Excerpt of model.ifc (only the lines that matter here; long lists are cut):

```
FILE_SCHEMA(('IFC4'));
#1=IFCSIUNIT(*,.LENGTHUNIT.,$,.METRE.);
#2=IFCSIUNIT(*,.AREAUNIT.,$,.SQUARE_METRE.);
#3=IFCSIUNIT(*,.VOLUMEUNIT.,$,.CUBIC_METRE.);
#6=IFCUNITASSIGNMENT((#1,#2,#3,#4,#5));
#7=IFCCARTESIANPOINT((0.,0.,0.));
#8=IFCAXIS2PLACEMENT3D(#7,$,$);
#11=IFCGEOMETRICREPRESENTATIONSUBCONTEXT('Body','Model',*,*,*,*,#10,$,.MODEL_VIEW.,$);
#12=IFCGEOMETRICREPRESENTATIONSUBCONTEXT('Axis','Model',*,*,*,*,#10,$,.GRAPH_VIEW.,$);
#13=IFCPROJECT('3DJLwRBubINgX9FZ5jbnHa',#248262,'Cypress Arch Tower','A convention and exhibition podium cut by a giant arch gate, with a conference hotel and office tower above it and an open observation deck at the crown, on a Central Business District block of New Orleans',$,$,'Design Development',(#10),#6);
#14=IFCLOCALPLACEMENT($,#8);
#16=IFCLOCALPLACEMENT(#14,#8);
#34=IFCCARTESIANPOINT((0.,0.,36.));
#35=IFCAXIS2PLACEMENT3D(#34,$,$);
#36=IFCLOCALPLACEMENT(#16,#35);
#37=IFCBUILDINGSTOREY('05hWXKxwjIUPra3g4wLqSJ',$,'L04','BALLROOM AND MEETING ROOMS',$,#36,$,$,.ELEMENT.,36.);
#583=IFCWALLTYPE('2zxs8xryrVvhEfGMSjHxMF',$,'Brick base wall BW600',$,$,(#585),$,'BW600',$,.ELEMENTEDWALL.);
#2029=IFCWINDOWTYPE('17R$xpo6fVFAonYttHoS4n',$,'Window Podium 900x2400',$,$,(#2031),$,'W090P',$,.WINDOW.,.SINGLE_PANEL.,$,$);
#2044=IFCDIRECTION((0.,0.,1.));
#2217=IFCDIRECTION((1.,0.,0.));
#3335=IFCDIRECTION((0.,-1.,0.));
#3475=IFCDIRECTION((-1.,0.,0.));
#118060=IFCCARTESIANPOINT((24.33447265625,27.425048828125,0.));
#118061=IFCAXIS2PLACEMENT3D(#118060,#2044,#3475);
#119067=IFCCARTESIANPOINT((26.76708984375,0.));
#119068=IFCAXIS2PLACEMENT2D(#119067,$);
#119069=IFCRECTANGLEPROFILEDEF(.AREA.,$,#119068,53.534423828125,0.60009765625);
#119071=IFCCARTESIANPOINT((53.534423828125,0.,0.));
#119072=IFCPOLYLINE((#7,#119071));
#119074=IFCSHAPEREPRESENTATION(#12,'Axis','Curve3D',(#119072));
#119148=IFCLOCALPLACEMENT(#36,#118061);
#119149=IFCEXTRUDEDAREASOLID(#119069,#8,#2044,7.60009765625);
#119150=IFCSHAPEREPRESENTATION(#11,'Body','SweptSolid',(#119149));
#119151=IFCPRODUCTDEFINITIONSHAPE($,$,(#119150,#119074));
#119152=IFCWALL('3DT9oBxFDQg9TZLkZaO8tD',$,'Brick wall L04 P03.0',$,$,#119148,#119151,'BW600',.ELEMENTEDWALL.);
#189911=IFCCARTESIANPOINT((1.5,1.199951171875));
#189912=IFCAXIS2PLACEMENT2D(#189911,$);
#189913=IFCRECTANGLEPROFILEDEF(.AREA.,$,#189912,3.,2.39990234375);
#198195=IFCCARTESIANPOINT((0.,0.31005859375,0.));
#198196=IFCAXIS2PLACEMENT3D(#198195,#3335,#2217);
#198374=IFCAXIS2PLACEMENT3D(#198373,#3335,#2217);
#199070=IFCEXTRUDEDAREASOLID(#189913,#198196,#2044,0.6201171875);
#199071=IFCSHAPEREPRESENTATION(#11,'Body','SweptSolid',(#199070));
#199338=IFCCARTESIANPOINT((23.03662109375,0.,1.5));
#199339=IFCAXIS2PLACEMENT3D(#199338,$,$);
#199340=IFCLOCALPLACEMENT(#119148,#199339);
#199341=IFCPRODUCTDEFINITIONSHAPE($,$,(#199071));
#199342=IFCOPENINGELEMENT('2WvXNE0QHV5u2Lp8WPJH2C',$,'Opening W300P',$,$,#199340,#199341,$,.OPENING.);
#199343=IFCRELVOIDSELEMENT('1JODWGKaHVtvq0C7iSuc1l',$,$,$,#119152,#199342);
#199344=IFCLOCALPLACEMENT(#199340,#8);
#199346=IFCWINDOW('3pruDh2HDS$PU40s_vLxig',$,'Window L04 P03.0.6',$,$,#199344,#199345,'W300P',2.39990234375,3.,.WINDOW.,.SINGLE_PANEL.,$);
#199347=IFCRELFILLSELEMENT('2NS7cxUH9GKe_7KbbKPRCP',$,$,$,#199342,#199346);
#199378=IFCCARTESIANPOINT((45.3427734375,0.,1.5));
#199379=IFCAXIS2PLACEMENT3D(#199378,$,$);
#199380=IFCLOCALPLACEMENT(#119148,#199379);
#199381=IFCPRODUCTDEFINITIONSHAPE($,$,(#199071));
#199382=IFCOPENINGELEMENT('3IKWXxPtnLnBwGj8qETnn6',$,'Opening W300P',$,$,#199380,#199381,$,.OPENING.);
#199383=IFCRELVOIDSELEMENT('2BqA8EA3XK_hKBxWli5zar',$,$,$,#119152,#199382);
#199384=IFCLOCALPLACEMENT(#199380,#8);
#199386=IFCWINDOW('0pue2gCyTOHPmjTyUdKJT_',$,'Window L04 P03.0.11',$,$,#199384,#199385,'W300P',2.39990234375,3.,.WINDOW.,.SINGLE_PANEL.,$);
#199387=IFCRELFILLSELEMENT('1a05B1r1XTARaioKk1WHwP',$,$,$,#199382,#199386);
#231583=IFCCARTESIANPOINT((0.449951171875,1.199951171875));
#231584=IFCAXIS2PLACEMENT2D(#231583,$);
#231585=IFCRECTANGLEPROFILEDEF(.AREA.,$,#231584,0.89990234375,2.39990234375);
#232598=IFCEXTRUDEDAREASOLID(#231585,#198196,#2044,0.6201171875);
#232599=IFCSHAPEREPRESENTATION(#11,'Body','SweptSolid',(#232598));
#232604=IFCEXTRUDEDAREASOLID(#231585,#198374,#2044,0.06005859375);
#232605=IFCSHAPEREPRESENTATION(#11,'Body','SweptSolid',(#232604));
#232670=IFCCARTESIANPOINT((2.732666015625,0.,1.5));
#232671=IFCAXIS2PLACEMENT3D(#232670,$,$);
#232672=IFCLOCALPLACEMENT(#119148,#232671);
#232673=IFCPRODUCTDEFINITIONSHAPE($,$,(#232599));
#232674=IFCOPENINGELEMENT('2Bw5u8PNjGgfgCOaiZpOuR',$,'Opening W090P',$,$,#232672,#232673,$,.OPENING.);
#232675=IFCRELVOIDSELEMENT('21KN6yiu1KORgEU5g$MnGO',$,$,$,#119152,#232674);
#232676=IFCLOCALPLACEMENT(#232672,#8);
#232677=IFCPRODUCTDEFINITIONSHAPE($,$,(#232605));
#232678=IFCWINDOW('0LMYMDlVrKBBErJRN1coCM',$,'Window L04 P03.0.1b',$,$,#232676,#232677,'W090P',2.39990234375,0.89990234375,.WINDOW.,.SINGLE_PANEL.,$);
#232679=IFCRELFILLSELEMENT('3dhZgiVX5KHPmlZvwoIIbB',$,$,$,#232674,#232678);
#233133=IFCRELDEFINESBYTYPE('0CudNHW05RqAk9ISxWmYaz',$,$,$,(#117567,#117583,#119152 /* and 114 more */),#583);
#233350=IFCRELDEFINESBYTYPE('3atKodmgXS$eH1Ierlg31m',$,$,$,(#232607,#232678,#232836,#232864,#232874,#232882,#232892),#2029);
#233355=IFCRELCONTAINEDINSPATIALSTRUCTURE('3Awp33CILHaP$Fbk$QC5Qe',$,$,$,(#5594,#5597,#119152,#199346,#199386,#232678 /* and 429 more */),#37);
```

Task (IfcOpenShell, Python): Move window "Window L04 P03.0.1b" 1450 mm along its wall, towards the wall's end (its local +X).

```python
import ifcopenshell
import ifcopenshell.api.geometry
import ifcopenshell.util.placement

model = ifcopenshell.open("model.ifc")

window = model.by_guid("0LMYMDlVrKBBErJRN1coCM")
opening = window.FillsVoids[0].RelatingOpeningElement
wall = opening.VoidsElements[0].RelatingBuildingElement

wall_matrix = ifcopenshell.util.placement.get_local_placement(wall.ObjectPlacement)
shift = wall_matrix[:3, 0] * 1.45
before = ifcopenshell.util.placement.get_local_placement(window.ObjectPlacement)[:3, 3].copy()

# The window is placed relative to its opening, so it follows when the opening moves.
matrix = ifcopenshell.util.placement.get_local_placement(opening.ObjectPlacement)
matrix[:3, 3] += shift
ifcopenshell.api.geometry.edit_object_placement(
    model, product=opening, matrix=matrix, is_si=False, should_transform_children=True
)

after = ifcopenshell.util.placement.get_local_placement(window.ObjectPlacement)[:3, 3]
print("window moved by", (after - before).round(3) + 0.0)

model.write("model_rev.ifc")
```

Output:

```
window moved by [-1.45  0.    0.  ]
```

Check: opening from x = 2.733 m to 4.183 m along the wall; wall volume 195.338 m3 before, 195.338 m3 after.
